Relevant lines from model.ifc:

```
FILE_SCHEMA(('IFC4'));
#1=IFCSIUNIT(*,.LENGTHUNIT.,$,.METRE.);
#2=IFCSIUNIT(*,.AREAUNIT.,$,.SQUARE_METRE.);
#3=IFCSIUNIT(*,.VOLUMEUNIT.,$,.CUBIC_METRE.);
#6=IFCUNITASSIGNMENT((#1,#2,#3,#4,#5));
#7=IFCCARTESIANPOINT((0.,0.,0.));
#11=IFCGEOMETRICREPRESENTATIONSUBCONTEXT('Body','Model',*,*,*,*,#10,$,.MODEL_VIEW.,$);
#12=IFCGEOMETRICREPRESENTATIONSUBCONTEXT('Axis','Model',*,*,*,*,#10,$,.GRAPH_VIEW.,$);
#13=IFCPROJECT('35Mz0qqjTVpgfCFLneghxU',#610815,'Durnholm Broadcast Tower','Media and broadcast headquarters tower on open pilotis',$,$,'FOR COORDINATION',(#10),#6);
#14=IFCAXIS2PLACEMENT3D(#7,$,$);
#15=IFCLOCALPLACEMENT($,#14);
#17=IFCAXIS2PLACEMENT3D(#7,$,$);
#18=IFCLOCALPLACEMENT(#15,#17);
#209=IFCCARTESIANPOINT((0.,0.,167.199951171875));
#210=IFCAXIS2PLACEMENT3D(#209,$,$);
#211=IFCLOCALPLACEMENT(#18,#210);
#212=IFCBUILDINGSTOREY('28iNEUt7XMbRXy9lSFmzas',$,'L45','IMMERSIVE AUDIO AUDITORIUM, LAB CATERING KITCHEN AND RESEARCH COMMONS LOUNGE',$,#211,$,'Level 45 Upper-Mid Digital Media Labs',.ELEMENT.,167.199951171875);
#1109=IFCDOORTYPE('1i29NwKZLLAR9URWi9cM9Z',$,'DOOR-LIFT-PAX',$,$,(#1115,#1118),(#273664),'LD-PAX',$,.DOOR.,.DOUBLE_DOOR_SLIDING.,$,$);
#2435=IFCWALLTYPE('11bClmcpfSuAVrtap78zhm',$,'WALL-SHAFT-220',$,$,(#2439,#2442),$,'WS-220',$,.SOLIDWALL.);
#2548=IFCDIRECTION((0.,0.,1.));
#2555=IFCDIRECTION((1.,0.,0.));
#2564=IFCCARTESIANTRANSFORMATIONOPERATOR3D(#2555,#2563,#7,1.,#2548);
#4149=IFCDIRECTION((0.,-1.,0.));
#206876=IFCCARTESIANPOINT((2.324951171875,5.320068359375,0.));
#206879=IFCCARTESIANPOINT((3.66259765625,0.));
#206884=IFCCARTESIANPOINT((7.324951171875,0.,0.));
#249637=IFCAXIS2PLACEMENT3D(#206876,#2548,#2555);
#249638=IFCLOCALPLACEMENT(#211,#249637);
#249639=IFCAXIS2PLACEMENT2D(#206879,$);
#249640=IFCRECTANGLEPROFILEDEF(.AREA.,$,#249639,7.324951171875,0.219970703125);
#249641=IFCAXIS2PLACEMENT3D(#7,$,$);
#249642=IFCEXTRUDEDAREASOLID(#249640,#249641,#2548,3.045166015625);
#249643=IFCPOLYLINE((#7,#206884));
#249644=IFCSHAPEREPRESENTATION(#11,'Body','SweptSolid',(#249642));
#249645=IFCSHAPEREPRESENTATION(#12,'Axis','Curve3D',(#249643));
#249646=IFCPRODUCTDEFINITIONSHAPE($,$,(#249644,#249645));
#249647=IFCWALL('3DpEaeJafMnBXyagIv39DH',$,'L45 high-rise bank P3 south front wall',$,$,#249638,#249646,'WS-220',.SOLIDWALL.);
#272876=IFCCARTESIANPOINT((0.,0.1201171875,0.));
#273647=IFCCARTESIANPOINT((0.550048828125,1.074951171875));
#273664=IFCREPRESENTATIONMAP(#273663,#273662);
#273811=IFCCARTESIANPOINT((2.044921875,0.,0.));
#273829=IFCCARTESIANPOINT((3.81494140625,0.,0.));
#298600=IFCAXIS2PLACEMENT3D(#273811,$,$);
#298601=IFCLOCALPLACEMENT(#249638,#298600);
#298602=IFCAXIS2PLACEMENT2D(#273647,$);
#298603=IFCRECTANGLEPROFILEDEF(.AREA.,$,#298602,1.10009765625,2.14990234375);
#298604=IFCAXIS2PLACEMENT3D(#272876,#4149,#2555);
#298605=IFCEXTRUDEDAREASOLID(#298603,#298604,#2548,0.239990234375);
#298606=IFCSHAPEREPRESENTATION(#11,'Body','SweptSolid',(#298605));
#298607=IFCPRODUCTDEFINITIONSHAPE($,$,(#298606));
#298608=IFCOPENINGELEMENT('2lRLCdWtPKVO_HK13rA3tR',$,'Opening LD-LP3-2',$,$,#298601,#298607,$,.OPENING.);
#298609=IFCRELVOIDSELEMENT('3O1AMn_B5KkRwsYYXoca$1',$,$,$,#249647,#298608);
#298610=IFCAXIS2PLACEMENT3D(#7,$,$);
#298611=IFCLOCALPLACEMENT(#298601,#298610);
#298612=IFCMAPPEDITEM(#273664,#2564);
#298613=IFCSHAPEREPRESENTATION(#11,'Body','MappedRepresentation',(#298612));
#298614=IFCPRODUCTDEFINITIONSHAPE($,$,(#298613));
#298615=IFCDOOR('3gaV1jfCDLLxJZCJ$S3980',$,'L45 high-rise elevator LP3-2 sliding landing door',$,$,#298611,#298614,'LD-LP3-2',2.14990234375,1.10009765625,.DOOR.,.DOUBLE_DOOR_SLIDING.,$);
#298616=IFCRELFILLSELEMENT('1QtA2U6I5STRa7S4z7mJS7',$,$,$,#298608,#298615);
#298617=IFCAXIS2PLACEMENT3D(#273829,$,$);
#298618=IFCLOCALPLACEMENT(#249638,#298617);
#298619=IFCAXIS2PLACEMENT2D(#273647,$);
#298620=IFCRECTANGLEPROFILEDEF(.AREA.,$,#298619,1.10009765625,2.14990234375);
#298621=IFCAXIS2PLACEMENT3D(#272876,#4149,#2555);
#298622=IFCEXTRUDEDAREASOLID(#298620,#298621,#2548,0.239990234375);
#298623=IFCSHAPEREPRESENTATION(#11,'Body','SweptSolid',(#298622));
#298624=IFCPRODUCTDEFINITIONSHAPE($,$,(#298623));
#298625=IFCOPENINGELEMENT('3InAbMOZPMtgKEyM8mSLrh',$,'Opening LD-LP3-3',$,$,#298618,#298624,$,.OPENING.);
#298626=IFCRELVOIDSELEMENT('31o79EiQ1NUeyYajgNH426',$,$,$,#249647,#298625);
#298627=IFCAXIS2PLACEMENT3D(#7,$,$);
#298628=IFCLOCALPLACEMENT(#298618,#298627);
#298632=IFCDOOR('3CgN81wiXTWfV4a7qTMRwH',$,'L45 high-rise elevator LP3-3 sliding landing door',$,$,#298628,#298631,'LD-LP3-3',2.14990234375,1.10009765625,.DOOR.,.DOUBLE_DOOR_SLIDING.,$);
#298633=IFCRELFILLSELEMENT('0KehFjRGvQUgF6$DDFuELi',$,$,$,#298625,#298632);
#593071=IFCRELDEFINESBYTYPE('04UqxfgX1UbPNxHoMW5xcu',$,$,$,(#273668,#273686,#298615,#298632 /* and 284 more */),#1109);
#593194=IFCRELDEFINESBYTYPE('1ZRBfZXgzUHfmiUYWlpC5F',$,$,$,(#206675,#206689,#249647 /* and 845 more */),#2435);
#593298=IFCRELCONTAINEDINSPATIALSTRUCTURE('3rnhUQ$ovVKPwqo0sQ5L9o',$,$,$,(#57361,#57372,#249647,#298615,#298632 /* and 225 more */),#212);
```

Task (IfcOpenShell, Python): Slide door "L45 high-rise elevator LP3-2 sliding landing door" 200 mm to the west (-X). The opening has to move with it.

```python
import ifcopenshell
import ifcopenshell.api.geometry
import ifcopenshell.util.placement
import ifcopenshell.util.unit

model = ifcopenshell.open("model.ifc")
unit_scale = ifcopenshell.util.unit.calculate_unit_scale(model)

door = model.by_guid("3gaV1jfCDLLxJZCJ$S3980")
opening = door.FillsVoids[0].RelatingOpeningElement
wall = opening.VoidsElements[0].RelatingBuildingElement

wall_matrix = ifcopenshell.util.placement.get_local_placement(wall.ObjectPlacement)
shift = wall_matrix[:3, 0] * -0.2 / unit_scale
before = ifcopenshell.util.placement.get_local_placement(door.ObjectPlacement)[:3, 3].copy()

# The door is placed relative to its opening, so it follows when the opening moves.
matrix = ifcopenshell.util.placement.get_local_placement(opening.ObjectPlacement)
matrix[:3, 3] += shift
ifcopenshell.api.geometry.edit_object_placement(
    model, product=opening, matrix=matrix, is_si=False, should_transform_children=True
)

after = ifcopenshell.util.placement.get_local_placement(door.ObjectPlacement)[:3, 3]
print("door moved by", (after - before).round(3) + 0.0)

model.write("model-out.ifc")
```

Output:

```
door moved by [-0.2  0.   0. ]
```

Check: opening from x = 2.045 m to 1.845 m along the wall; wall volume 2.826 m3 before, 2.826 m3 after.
